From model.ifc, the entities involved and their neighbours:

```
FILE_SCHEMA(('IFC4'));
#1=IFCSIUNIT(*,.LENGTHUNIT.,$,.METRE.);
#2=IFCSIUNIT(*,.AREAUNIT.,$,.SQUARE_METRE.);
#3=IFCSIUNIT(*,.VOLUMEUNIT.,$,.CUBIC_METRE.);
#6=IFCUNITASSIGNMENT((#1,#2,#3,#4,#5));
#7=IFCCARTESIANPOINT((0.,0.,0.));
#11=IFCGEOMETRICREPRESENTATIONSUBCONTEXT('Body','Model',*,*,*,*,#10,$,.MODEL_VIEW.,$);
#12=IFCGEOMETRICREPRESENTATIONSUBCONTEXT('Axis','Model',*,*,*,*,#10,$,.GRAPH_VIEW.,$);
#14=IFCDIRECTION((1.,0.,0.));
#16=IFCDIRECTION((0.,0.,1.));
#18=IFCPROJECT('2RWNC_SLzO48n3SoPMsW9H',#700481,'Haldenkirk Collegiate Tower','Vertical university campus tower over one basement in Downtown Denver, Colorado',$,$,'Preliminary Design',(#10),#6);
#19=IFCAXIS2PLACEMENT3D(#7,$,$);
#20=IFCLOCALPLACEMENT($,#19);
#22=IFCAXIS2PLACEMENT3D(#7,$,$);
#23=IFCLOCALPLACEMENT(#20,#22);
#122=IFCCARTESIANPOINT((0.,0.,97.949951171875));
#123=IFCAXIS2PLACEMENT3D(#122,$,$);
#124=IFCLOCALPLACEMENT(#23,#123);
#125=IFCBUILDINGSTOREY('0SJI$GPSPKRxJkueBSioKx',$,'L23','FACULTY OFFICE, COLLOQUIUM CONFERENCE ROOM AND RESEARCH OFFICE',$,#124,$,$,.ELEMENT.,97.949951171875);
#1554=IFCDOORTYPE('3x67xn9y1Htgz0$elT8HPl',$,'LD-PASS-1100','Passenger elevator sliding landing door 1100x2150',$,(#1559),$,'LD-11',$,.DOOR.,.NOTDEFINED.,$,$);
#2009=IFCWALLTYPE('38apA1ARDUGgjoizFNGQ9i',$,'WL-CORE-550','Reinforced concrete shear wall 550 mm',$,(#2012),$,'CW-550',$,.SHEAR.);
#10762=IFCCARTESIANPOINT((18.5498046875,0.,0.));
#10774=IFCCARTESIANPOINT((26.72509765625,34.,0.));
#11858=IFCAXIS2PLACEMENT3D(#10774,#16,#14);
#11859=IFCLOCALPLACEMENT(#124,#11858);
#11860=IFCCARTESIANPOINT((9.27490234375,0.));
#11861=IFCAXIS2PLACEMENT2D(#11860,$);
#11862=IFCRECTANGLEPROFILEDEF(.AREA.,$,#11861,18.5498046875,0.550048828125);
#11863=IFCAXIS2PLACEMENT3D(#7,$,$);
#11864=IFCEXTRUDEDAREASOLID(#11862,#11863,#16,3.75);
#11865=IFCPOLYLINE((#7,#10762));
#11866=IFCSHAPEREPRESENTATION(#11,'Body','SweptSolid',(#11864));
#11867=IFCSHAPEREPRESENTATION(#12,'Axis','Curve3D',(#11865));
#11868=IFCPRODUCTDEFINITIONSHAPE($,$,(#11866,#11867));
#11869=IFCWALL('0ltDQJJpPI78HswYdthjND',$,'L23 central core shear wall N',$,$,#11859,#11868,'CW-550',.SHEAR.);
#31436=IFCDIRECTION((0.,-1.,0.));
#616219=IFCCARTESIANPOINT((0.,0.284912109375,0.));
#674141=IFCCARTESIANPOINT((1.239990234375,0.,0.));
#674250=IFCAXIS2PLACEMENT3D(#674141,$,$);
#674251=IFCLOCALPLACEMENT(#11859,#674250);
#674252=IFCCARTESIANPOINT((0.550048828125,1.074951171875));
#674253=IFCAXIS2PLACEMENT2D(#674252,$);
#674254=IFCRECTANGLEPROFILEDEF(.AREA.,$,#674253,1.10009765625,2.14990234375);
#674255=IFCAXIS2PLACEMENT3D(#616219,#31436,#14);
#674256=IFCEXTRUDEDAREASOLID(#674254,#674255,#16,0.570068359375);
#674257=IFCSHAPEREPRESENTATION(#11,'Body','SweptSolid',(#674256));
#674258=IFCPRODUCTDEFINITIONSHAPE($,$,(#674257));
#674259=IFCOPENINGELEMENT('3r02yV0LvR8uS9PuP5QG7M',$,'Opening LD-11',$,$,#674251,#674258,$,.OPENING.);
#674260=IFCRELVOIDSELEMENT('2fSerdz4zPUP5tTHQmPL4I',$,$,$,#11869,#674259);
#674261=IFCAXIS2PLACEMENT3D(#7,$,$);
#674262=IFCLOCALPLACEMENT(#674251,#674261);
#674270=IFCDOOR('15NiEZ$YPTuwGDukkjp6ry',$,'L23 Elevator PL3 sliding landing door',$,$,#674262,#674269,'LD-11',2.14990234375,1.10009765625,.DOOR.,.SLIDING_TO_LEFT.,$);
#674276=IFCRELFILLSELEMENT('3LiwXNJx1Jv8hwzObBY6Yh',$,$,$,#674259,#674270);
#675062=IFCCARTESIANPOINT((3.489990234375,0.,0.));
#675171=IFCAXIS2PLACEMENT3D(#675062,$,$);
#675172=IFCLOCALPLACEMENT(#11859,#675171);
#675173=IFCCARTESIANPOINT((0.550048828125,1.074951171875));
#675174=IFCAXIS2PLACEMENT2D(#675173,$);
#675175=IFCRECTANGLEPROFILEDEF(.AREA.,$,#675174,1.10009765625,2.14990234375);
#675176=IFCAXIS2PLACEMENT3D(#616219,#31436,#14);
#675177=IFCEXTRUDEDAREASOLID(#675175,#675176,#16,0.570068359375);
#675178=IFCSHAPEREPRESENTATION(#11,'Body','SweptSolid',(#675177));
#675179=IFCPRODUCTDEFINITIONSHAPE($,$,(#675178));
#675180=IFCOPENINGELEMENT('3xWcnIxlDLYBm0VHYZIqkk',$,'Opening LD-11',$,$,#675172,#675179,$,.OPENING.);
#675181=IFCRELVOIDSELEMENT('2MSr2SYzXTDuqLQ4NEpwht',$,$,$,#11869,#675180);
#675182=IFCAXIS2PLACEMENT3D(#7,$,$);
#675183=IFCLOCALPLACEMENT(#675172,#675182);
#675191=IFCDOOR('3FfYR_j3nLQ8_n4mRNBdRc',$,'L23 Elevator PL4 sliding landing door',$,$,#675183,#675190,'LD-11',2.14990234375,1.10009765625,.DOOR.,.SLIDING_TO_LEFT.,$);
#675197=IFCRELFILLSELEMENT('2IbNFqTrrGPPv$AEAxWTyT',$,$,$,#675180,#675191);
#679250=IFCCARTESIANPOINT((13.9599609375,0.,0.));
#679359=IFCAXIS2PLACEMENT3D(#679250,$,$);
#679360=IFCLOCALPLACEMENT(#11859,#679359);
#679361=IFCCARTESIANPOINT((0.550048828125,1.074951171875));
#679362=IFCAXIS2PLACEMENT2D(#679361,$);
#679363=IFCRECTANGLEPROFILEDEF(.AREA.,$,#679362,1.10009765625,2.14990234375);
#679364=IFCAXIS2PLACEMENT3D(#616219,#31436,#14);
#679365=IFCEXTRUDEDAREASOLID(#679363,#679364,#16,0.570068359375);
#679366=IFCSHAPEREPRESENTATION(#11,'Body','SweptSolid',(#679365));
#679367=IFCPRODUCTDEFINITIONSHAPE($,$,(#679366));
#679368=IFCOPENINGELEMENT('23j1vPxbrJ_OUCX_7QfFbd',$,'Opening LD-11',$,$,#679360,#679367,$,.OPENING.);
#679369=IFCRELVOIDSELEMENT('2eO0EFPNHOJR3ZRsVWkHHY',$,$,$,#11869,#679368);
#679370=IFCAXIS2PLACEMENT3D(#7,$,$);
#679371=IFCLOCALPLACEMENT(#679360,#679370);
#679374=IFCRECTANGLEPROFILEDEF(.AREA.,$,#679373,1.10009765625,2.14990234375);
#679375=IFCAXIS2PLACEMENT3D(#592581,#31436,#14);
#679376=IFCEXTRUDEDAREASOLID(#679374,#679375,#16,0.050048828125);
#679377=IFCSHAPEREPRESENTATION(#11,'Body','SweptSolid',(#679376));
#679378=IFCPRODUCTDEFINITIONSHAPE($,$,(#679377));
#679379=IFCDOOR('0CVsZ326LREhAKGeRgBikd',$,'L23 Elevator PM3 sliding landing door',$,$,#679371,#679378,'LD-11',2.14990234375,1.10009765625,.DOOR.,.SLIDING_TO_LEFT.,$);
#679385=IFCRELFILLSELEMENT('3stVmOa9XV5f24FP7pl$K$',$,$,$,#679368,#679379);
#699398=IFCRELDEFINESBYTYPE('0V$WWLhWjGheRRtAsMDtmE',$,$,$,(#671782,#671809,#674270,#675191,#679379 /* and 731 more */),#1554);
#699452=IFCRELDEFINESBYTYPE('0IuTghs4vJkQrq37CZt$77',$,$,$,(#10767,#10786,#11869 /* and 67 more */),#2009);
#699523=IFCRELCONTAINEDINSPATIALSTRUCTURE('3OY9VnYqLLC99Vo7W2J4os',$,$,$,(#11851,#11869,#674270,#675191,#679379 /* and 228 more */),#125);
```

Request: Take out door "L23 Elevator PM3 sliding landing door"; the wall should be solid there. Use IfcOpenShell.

```python
import ifcopenshell
import ifcopenshell.api.feature
import ifcopenshell.api.root
import ifcopenshell.geom
import ifcopenshell.util.shape

model = ifcopenshell.open("model.ifc")
settings = ifcopenshell.geom.settings()


def volume(element):
    """Net volume in cubic metres, openings subtracted."""
    shape = ifcopenshell.geom.create_shape(settings, element)
    return ifcopenshell.util.shape.get_volume(shape.geometry)


door = model.by_id(679379)
opening = door.FillsVoids[0].RelatingOpeningElement
wall = opening.VoidsElements[0].RelatingBuildingElement
before = volume(wall)

ifcopenshell.api.root.remove_product(model, product=door)
ifcopenshell.api.feature.remove_feature(model, feature=opening)

after = volume(wall)

print(f"wall volume {before:.3f} -> {after:.3f} m3")

model.write("model_v2.ifc")
```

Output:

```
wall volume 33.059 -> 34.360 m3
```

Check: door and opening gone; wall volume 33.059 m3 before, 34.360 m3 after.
